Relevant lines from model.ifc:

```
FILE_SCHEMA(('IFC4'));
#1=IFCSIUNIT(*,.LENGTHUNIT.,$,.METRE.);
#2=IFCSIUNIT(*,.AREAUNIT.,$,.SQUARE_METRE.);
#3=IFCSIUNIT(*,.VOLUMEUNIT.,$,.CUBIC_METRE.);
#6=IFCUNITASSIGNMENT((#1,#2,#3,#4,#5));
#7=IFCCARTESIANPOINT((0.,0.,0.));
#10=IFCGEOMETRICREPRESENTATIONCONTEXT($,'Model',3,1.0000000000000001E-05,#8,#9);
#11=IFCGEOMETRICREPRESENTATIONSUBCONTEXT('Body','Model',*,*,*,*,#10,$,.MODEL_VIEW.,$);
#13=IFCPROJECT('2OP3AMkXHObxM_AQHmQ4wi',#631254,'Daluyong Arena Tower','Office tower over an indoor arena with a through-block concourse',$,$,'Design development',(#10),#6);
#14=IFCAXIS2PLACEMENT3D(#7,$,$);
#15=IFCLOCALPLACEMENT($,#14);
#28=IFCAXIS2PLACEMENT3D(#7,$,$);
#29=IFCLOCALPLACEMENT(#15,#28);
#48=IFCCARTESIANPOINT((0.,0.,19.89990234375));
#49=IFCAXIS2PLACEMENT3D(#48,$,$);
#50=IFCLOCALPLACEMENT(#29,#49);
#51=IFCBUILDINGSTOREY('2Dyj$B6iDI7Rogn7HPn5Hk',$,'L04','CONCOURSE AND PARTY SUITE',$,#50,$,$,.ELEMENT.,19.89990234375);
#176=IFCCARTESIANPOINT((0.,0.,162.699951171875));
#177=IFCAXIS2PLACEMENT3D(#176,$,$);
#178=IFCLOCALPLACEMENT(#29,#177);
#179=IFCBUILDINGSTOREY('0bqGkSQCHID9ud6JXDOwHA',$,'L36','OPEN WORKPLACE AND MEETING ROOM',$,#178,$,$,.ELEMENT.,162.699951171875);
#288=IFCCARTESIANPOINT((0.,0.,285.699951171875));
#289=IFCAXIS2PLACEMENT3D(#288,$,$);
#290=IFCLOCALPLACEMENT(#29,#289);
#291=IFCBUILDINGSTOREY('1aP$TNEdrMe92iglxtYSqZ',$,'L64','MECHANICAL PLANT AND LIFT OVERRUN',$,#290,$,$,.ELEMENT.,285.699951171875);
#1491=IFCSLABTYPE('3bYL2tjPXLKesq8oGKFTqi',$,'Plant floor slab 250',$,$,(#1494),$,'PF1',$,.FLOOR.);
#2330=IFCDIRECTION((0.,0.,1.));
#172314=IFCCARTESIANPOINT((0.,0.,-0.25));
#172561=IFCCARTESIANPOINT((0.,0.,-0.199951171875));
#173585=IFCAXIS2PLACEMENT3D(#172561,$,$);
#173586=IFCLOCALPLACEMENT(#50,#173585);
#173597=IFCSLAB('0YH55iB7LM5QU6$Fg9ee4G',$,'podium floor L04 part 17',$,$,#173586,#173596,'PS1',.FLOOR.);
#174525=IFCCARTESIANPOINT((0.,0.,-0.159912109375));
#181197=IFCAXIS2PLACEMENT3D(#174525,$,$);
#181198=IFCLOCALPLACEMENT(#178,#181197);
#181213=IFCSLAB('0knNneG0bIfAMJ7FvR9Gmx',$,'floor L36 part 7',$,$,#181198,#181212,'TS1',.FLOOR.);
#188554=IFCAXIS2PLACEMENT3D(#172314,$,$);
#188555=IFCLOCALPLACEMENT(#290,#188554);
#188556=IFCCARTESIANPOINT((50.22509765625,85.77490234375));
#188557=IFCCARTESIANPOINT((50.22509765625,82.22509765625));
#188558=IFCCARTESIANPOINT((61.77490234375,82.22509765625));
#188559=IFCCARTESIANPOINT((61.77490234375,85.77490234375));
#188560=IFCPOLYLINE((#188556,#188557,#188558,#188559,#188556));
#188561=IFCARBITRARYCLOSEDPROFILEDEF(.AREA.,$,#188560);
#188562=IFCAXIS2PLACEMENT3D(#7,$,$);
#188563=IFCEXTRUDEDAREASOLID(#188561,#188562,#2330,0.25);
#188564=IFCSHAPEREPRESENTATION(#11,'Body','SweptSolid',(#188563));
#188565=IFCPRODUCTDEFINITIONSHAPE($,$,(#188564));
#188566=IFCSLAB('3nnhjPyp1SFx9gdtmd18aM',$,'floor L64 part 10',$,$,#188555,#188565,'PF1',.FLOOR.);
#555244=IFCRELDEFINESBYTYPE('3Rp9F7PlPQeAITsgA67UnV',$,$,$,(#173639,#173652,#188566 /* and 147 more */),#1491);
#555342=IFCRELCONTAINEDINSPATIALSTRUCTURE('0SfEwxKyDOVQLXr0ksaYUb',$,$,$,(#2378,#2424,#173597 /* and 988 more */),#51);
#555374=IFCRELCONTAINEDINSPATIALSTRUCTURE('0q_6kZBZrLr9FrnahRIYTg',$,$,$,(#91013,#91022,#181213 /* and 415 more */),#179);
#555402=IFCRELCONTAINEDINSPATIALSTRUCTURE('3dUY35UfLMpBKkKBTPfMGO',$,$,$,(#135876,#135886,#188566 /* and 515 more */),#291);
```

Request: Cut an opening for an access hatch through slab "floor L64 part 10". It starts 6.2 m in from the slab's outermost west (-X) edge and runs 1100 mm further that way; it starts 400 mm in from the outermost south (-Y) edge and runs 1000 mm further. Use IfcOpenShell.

```python
import numpy as np
import ifcopenshell
import ifcopenshell.api.feature
import ifcopenshell.api.geometry
import ifcopenshell.api.root
import ifcopenshell.geom
import ifcopenshell.util.placement
import ifcopenshell.util.representation
import ifcopenshell.util.shape
import ifcopenshell.util.unit

model = ifcopenshell.open("model.ifc")
unit_scale = ifcopenshell.util.unit.calculate_unit_scale(model)
settings = ifcopenshell.geom.settings()


def volume(element):
    """Net volume in cubic metres, openings subtracted."""
    shape = ifcopenshell.geom.create_shape(settings, element)
    return ifcopenshell.util.shape.get_volume(shape.geometry)


slab = model.by_guid("3nnhjPyp1SFx9gdtmd18aM")
before = volume(slab)

# Extent in the slab's own axes, in metres. The edges named are its -X and -Y sides.
slab_shape = ifcopenshell.geom.create_shape(settings, slab)
vertices = ifcopenshell.util.shape.get_vertices(slab_shape.geometry)
x_min, y_min, bottom = vertices.min(axis=0)
top = vertices[:, 2].max()

opening = ifcopenshell.api.root.create_entity(model, ifc_class="IfcOpeningElement", name="Access hatch opening", predefined_type="OPENING")
context = ifcopenshell.util.representation.get_context(model, "Model", "Body", "MODEL_VIEW")
width, depth = 1.1, 1
outline = [(0.0, 0.0), (width, 0.0), (width, depth), (0.0, depth), (0.0, 0.0)]
# Overshoot both faces by 50 mm so the cut is clean.
shape = ifcopenshell.api.geometry.add_slab_representation(
    model, context=context, depth=top - bottom + 0.1, polyline=outline
)
ifcopenshell.api.geometry.assign_representation(model, product=opening, representation=shape)

matrix = ifcopenshell.util.placement.get_local_placement(slab.ObjectPlacement)
matrix[:, 3] = matrix @ np.append(np.array([x_min + 6.2, y_min + 0.4, bottom - 0.05]) / unit_scale, 1.0)
ifcopenshell.api.geometry.edit_object_placement(model, product=opening, matrix=matrix, is_si=False)
ifcopenshell.api.feature.add_feature(model, feature=opening, element=slab)

after = volume(slab)

print(f"slab volume {before:.3f} -> {after:.3f} m3")

model.write("model_v2.ifc")
```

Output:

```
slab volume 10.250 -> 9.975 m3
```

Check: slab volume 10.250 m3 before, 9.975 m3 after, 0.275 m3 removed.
